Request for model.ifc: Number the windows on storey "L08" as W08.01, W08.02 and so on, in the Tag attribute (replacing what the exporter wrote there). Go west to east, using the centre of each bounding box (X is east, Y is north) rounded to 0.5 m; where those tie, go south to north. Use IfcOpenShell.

First a look at what the model holds.

```python
import ifcopenshell
import ifcopenshell.util.element
import ifcopenshell.util.placement

model = ifcopenshell.open("model.ifc")
print(model.schema)
storey = next(s for s in model.by_type("IfcBuildingStorey") if s.Name == "L08")
windows = [e for e in ifcopenshell.util.element.get_decomposition(storey) if e.is_a("IfcWindow")]
for e in sorted(windows, key=lambda e: e.id()):
    origin = ifcopenshell.util.placement.get_local_placement(e.ObjectPlacement)[:3, 3]
    print(e.id(), e.Tag, e.Name, origin.round(2) + 0.0, sep=" | ")
```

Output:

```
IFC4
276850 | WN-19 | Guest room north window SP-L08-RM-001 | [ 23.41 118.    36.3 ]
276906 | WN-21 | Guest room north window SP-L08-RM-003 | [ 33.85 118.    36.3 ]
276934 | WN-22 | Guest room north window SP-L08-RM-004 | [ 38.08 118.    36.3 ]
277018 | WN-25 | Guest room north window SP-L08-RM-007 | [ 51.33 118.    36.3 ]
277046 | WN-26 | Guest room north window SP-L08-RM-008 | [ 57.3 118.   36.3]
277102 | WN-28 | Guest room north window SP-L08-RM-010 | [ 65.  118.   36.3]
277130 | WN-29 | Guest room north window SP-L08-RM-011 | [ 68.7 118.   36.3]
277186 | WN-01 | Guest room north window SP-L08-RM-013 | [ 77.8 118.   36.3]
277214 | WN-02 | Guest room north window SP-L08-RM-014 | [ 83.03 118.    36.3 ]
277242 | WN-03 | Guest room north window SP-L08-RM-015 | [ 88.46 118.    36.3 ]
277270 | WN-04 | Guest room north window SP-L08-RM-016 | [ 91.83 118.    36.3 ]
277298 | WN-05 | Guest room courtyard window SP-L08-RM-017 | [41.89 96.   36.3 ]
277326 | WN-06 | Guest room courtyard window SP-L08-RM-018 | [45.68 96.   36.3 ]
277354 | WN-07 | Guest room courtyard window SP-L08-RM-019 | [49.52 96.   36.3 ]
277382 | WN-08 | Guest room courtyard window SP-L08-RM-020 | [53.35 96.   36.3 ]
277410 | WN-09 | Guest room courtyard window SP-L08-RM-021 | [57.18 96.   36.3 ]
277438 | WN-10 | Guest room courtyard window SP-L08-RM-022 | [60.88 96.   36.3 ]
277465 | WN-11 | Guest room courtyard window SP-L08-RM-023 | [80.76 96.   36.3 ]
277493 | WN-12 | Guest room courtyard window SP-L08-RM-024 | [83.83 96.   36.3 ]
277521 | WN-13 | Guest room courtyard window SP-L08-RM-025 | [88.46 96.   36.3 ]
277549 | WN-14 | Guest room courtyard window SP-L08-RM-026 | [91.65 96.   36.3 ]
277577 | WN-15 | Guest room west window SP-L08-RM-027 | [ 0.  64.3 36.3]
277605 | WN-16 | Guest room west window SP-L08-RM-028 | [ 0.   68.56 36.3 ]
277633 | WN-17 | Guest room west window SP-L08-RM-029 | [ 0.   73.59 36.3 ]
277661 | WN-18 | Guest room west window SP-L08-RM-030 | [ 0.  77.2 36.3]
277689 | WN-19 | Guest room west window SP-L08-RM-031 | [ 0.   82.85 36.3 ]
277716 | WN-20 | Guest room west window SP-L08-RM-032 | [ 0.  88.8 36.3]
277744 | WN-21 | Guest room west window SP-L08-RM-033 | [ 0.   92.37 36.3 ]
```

```python
import ifcopenshell
import ifcopenshell.geom
import ifcopenshell.util.element
import ifcopenshell.util.shape

model = ifcopenshell.open("model.ifc")
settings = ifcopenshell.geom.settings()
settings.set("use-world-coords", True)


def centre(element):
    shape = ifcopenshell.geom.create_shape(settings, element)
    return ifcopenshell.util.shape.get_bbox_centroid(shape.geometry)


storey = next(s for s in model.by_type("IfcBuildingStorey") if s.Name == "L08")
windows = [e for e in ifcopenshell.util.element.get_decomposition(storey) if e.is_a("IfcWindow")]

# Insertion points can sit at a corner or the storey origin, so sort by the geometry (in metres).
centres = {e: centre(e) for e in windows}
windows.sort(key=lambda e: (round(centres[e][0] / 0.5), centres[e][1]))

for i, e in enumerate(windows, start=1):
    number = f"W08.{i:02d}"
    e.Tag = number
    print(e.id(), number)

model.write("model_rev.ifc")
```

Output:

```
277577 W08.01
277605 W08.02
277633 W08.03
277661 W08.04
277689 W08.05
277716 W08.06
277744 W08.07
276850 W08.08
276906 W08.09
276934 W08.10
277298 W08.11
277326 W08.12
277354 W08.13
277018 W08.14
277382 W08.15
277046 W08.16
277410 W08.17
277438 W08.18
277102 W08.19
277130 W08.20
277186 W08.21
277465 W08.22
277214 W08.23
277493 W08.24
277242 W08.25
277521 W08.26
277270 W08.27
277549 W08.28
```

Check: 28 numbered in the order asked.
